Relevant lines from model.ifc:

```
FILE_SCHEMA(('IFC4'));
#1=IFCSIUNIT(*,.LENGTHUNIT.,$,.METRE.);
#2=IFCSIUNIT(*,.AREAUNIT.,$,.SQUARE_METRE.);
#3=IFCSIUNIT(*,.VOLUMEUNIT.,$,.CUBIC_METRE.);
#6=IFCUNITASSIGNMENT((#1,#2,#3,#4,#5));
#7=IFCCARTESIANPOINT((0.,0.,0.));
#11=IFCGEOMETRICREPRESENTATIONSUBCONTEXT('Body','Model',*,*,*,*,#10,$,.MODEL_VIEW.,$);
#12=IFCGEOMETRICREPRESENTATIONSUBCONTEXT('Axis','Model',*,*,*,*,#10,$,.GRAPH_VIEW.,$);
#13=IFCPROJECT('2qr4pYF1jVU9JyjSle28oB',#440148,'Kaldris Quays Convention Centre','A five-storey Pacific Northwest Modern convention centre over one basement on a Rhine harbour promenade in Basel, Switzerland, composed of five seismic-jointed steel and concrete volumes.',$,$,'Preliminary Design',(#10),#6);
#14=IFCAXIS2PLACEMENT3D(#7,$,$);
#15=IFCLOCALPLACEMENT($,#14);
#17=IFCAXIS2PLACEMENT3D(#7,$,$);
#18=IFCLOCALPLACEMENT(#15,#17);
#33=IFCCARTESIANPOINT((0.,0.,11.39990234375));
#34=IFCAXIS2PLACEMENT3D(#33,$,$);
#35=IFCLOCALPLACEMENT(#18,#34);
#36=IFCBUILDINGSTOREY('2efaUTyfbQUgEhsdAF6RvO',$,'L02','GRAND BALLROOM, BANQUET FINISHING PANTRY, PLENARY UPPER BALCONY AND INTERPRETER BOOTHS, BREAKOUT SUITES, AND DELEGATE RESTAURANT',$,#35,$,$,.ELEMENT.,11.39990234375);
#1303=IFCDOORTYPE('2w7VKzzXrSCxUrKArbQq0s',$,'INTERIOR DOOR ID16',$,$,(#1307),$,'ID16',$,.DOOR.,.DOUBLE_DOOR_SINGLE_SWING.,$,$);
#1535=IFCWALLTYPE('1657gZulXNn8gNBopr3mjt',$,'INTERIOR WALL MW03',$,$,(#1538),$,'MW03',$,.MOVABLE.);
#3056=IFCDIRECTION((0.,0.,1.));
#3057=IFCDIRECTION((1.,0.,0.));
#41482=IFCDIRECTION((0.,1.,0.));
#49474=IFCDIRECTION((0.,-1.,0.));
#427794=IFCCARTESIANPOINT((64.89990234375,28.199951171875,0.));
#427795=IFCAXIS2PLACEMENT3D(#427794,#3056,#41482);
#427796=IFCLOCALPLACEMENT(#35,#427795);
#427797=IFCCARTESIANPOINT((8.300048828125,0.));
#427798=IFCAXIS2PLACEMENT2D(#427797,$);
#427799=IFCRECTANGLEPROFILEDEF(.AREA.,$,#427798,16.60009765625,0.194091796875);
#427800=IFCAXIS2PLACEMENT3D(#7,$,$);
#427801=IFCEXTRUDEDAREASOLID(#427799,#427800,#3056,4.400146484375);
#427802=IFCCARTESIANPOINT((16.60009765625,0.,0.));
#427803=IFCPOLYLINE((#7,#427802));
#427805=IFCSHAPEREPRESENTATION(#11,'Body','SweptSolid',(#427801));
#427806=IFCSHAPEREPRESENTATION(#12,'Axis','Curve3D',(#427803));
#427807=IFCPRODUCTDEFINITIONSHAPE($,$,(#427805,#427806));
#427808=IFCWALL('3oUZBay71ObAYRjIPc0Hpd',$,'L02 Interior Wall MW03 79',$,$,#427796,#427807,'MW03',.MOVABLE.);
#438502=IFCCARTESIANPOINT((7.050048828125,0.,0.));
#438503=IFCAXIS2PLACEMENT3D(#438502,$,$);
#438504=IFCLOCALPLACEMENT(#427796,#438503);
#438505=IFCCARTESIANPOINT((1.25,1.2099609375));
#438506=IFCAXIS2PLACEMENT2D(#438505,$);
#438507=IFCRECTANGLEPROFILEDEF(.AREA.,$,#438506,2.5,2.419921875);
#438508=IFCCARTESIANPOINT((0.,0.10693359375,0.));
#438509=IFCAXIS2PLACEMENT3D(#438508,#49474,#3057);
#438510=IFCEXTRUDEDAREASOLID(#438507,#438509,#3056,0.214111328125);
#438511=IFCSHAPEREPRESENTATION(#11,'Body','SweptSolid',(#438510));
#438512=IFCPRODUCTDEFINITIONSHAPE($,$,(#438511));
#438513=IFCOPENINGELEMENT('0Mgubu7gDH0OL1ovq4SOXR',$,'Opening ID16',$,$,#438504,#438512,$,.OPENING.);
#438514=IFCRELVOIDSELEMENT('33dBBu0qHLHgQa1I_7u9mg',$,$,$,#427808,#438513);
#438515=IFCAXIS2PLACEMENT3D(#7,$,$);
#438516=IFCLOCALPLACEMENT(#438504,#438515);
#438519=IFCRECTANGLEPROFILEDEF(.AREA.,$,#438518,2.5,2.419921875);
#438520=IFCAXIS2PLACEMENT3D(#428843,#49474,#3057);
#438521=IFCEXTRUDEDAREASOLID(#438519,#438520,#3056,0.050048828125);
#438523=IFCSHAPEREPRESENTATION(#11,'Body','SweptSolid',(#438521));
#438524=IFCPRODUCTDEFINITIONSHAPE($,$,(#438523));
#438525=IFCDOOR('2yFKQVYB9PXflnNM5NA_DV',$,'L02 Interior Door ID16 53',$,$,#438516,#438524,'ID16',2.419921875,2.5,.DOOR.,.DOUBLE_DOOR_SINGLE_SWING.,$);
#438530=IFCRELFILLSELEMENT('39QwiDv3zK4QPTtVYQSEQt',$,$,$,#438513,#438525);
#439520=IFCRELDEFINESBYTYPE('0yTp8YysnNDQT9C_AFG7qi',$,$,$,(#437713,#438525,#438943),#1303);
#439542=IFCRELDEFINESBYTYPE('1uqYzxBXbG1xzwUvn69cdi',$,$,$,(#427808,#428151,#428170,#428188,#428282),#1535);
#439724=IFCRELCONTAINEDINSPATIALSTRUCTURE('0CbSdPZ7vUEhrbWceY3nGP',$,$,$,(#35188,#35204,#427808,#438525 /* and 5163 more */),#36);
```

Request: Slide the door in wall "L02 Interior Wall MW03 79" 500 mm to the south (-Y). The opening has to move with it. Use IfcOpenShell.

```python
import ifcopenshell
import ifcopenshell.api.geometry
import ifcopenshell.util.placement
import ifcopenshell.util.unit

model = ifcopenshell.open("model.ifc")
unit_scale = ifcopenshell.util.unit.calculate_unit_scale(model)

door = model.by_guid("2yFKQVYB9PXflnNM5NA_DV")
opening = door.FillsVoids[0].RelatingOpeningElement
wall = opening.VoidsElements[0].RelatingBuildingElement

wall_matrix = ifcopenshell.util.placement.get_local_placement(wall.ObjectPlacement)
shift = wall_matrix[:3, 0] * -0.5 / unit_scale
before = ifcopenshell.util.placement.get_local_placement(door.ObjectPlacement)[:3, 3].copy()

# The door is placed relative to its opening, so it follows when the opening moves.
matrix = ifcopenshell.util.placement.get_local_placement(opening.ObjectPlacement)
matrix[:3, 3] += shift
ifcopenshell.api.geometry.edit_object_placement(
    model, product=opening, matrix=matrix, is_si=False, should_transform_children=True
)

after = ifcopenshell.util.placement.get_local_placement(door.ObjectPlacement)[:3, 3]
print("door moved by", (after - before).round(3) + 0.0)

model.write("model-out.ifc")
```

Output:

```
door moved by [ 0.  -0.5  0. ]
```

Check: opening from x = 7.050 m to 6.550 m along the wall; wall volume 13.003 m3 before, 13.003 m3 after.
